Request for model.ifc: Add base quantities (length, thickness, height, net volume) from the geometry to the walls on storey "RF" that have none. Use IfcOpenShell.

First a look at what the model holds.

```python
import ifcopenshell
import ifcopenshell.util.element
import ifcopenshell.util.unit

model = ifcopenshell.open("model.ifc")
print(model.schema)
for unit_type in ("LENGTHUNIT", "AREAUNIT", "VOLUMEUNIT"):
    print(unit_type, ifcopenshell.util.unit.calculate_unit_scale(model, unit_type))
storey = next(s for s in model.by_type("IfcBuildingStorey") if s.Name == "RF")
walls = [e for e in ifcopenshell.util.element.get_decomposition(storey) if e.is_a("IfcWall")]
for e in sorted(walls, key=lambda e: e.id()):
    print(e.id(), e.is_a(), e.Name, list(ifcopenshell.util.element.get_psets(e, qtos_only=True)), sep=" | ")
```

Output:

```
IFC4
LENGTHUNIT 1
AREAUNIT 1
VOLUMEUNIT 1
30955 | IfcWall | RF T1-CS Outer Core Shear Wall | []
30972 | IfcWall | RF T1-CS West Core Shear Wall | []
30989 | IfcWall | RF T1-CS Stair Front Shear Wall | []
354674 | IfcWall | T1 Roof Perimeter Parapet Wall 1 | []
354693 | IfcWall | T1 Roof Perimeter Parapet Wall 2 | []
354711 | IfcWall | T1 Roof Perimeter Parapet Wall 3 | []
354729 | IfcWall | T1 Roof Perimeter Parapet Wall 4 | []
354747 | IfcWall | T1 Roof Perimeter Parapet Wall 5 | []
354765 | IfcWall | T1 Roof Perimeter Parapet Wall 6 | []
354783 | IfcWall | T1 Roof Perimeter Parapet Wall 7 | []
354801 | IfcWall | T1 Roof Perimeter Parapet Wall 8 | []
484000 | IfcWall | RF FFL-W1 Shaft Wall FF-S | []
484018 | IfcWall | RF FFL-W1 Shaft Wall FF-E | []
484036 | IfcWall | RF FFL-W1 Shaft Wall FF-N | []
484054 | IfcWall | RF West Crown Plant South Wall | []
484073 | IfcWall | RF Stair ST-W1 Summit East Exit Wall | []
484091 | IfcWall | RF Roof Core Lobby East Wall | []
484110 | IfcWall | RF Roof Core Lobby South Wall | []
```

```python
import ifcopenshell
import ifcopenshell.api.pset
import ifcopenshell.geom
import ifcopenshell.util.element
import ifcopenshell.util.shape
import ifcopenshell.util.unit

model = ifcopenshell.open("model.ifc")
unit_scale = ifcopenshell.util.unit.calculate_unit_scale(model)
volume_scale = ifcopenshell.util.unit.calculate_unit_scale(model, "VOLUMEUNIT")
settings = ifcopenshell.geom.settings()

storey = next(s for s in model.by_type("IfcBuildingStorey") if s.Name == "RF")
walls = [e for e in ifcopenshell.util.element.get_decomposition(storey) if e.is_a("IfcWall")]

for e in sorted(walls, key=lambda e: e.id()):
    if ifcopenshell.util.element.get_psets(e, qtos_only=True, should_inherit=False):
        continue
    # Geometry comes back in metres, in the element's own axes.
    shape = ifcopenshell.geom.create_shape(settings, e)
    values = {
        "Length": ifcopenshell.util.shape.get_x(shape.geometry) / unit_scale,
        "Width": ifcopenshell.util.shape.get_y(shape.geometry) / unit_scale,
        "Height": ifcopenshell.util.shape.get_z(shape.geometry) / unit_scale,
        "NetVolume": ifcopenshell.util.shape.get_volume(shape.geometry) / volume_scale,
    }
    qto = ifcopenshell.api.pset.add_qto(model, product=e, name="Qto_WallBaseQuantities")
    ifcopenshell.api.pset.edit_qto(model, qto=qto, properties=values)
    print(e.id(), {k: round(v, 3) for k, v in values.items()})

model.write("model_edited.ifc")
```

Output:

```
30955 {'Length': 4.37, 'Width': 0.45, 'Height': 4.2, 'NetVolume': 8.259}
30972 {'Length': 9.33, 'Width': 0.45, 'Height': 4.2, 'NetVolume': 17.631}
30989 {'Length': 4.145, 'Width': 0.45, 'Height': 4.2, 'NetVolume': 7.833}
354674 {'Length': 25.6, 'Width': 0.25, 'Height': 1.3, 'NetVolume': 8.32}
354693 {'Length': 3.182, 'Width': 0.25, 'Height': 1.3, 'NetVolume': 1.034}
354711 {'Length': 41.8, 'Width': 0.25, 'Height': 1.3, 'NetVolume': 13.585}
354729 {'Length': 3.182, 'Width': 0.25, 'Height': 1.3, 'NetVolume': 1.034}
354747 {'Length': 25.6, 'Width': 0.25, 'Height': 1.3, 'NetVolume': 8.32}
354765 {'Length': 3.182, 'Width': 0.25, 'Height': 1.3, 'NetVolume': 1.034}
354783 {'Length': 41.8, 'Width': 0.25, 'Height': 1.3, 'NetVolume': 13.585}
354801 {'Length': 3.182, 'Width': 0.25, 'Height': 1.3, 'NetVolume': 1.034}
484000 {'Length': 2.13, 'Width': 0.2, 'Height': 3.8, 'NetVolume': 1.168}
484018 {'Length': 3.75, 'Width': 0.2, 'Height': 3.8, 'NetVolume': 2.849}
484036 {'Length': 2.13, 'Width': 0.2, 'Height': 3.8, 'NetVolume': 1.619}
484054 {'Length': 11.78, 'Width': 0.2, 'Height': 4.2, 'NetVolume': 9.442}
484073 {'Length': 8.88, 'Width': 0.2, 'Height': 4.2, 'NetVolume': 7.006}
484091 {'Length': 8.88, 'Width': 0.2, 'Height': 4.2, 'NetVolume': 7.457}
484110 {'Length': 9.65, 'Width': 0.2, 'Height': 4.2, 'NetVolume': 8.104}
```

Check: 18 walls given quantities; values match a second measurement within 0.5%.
